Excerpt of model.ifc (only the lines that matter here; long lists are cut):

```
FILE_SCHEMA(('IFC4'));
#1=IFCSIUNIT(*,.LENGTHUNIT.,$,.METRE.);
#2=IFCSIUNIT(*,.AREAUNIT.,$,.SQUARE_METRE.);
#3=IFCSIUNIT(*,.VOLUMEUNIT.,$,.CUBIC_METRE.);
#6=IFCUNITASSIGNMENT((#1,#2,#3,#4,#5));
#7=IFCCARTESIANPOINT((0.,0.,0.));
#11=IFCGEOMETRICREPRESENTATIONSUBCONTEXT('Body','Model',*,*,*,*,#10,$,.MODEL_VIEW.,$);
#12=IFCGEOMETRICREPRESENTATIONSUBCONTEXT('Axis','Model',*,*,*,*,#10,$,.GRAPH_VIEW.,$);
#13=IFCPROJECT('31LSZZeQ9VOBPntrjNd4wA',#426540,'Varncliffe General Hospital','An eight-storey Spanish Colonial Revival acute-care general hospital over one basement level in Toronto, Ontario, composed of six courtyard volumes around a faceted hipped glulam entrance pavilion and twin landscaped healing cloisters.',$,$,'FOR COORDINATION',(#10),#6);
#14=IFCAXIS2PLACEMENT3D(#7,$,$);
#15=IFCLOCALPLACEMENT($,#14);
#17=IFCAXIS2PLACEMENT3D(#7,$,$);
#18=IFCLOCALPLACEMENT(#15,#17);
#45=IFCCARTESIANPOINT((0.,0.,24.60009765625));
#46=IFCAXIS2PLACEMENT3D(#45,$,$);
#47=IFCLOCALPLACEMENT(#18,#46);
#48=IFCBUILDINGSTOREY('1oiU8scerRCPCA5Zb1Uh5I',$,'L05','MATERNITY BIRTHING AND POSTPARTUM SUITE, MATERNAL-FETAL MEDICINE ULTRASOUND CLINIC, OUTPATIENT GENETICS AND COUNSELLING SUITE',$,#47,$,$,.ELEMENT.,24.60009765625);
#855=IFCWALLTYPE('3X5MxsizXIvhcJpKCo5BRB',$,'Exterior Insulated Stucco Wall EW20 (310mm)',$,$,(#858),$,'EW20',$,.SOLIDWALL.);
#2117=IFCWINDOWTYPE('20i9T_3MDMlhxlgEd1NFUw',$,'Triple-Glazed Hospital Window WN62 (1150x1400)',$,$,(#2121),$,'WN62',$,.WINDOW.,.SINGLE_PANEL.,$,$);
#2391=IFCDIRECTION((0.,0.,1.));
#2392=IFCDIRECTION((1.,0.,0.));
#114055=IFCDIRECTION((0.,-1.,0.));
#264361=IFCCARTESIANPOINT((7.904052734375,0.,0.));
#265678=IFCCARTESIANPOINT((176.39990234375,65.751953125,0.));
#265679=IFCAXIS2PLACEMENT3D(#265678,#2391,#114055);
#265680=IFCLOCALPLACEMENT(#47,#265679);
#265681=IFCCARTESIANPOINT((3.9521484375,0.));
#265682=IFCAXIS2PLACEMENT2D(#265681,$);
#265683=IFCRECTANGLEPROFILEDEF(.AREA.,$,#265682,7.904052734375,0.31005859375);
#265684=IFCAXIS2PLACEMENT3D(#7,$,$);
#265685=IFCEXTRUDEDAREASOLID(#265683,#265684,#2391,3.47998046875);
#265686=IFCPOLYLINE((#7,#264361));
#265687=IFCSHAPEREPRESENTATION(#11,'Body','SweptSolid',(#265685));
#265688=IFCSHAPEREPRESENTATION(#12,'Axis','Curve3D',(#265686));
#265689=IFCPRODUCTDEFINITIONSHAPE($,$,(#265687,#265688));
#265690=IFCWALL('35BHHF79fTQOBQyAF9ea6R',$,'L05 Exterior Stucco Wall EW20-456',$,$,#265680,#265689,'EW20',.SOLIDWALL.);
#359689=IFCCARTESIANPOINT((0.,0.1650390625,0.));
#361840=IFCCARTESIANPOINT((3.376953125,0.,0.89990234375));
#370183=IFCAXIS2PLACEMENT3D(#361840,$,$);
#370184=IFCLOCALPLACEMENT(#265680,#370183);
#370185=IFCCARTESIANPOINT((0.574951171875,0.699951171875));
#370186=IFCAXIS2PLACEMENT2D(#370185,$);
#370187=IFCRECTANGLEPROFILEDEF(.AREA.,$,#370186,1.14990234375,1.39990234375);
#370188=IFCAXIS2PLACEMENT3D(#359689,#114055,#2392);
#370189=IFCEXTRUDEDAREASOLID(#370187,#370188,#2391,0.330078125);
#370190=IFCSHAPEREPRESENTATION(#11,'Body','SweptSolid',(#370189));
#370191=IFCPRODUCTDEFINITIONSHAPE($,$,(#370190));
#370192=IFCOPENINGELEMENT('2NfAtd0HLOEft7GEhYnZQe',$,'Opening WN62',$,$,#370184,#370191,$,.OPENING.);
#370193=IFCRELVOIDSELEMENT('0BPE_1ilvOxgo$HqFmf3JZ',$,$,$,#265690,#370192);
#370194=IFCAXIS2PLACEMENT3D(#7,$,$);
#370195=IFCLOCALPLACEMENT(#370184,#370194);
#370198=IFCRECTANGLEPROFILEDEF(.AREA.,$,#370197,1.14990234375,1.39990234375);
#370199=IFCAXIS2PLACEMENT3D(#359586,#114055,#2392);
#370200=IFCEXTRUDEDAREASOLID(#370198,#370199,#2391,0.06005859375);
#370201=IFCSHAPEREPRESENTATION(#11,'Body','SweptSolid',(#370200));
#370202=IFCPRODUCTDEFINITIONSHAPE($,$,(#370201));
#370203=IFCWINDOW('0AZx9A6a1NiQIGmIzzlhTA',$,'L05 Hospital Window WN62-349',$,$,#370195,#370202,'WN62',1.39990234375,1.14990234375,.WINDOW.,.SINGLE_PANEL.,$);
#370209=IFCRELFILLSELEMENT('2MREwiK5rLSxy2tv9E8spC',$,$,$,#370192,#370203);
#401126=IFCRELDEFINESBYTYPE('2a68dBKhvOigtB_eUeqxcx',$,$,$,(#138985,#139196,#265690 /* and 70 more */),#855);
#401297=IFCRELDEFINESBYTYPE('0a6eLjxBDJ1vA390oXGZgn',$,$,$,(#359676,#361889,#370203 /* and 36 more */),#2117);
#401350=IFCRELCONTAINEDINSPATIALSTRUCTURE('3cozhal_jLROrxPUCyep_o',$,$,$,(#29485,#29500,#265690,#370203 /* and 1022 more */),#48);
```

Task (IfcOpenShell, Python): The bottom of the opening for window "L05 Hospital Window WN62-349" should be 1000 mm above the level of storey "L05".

```python
import numpy as np
import ifcopenshell
import ifcopenshell.api.geometry
import ifcopenshell.geom
import ifcopenshell.util.element
import ifcopenshell.util.placement
import ifcopenshell.util.shape
import ifcopenshell.util.unit

model = ifcopenshell.open("model.ifc")
unit_scale = ifcopenshell.util.unit.calculate_unit_scale(model)

window = model.by_guid("0AZx9A6a1NiQIGmIzzlhTA")
opening = window.FillsVoids[0].RelatingOpeningElement
storey = ifcopenshell.util.element.get_container(window, ifc_class="IfcBuildingStorey")
level = ifcopenshell.util.placement.get_local_placement(storey.ObjectPlacement)[2, 3]

# The opening's origin need not be at the sill, so measure its lowest point.
shape = ifcopenshell.geom.create_shape(ifcopenshell.geom.settings(), opening)
bottom = ifcopenshell.util.shape.get_shape_bottom_elevation(shape, shape.geometry) / unit_scale
dz = level + 1 / unit_scale - bottom

shift = np.array([0.0, 0.0, dz])
# The window is placed relative to its opening, so it follows when the opening moves.
matrix = ifcopenshell.util.placement.get_local_placement(opening.ObjectPlacement)
matrix[:3, 3] += shift
ifcopenshell.api.geometry.edit_object_placement(
    model, product=opening, matrix=matrix, is_si=False, should_transform_children=True
)

print(f"moved by {dz * unit_scale:+.3f} m")

model.write("model_edited.ifc")
```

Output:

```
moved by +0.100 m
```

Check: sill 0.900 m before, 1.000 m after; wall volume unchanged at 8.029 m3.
